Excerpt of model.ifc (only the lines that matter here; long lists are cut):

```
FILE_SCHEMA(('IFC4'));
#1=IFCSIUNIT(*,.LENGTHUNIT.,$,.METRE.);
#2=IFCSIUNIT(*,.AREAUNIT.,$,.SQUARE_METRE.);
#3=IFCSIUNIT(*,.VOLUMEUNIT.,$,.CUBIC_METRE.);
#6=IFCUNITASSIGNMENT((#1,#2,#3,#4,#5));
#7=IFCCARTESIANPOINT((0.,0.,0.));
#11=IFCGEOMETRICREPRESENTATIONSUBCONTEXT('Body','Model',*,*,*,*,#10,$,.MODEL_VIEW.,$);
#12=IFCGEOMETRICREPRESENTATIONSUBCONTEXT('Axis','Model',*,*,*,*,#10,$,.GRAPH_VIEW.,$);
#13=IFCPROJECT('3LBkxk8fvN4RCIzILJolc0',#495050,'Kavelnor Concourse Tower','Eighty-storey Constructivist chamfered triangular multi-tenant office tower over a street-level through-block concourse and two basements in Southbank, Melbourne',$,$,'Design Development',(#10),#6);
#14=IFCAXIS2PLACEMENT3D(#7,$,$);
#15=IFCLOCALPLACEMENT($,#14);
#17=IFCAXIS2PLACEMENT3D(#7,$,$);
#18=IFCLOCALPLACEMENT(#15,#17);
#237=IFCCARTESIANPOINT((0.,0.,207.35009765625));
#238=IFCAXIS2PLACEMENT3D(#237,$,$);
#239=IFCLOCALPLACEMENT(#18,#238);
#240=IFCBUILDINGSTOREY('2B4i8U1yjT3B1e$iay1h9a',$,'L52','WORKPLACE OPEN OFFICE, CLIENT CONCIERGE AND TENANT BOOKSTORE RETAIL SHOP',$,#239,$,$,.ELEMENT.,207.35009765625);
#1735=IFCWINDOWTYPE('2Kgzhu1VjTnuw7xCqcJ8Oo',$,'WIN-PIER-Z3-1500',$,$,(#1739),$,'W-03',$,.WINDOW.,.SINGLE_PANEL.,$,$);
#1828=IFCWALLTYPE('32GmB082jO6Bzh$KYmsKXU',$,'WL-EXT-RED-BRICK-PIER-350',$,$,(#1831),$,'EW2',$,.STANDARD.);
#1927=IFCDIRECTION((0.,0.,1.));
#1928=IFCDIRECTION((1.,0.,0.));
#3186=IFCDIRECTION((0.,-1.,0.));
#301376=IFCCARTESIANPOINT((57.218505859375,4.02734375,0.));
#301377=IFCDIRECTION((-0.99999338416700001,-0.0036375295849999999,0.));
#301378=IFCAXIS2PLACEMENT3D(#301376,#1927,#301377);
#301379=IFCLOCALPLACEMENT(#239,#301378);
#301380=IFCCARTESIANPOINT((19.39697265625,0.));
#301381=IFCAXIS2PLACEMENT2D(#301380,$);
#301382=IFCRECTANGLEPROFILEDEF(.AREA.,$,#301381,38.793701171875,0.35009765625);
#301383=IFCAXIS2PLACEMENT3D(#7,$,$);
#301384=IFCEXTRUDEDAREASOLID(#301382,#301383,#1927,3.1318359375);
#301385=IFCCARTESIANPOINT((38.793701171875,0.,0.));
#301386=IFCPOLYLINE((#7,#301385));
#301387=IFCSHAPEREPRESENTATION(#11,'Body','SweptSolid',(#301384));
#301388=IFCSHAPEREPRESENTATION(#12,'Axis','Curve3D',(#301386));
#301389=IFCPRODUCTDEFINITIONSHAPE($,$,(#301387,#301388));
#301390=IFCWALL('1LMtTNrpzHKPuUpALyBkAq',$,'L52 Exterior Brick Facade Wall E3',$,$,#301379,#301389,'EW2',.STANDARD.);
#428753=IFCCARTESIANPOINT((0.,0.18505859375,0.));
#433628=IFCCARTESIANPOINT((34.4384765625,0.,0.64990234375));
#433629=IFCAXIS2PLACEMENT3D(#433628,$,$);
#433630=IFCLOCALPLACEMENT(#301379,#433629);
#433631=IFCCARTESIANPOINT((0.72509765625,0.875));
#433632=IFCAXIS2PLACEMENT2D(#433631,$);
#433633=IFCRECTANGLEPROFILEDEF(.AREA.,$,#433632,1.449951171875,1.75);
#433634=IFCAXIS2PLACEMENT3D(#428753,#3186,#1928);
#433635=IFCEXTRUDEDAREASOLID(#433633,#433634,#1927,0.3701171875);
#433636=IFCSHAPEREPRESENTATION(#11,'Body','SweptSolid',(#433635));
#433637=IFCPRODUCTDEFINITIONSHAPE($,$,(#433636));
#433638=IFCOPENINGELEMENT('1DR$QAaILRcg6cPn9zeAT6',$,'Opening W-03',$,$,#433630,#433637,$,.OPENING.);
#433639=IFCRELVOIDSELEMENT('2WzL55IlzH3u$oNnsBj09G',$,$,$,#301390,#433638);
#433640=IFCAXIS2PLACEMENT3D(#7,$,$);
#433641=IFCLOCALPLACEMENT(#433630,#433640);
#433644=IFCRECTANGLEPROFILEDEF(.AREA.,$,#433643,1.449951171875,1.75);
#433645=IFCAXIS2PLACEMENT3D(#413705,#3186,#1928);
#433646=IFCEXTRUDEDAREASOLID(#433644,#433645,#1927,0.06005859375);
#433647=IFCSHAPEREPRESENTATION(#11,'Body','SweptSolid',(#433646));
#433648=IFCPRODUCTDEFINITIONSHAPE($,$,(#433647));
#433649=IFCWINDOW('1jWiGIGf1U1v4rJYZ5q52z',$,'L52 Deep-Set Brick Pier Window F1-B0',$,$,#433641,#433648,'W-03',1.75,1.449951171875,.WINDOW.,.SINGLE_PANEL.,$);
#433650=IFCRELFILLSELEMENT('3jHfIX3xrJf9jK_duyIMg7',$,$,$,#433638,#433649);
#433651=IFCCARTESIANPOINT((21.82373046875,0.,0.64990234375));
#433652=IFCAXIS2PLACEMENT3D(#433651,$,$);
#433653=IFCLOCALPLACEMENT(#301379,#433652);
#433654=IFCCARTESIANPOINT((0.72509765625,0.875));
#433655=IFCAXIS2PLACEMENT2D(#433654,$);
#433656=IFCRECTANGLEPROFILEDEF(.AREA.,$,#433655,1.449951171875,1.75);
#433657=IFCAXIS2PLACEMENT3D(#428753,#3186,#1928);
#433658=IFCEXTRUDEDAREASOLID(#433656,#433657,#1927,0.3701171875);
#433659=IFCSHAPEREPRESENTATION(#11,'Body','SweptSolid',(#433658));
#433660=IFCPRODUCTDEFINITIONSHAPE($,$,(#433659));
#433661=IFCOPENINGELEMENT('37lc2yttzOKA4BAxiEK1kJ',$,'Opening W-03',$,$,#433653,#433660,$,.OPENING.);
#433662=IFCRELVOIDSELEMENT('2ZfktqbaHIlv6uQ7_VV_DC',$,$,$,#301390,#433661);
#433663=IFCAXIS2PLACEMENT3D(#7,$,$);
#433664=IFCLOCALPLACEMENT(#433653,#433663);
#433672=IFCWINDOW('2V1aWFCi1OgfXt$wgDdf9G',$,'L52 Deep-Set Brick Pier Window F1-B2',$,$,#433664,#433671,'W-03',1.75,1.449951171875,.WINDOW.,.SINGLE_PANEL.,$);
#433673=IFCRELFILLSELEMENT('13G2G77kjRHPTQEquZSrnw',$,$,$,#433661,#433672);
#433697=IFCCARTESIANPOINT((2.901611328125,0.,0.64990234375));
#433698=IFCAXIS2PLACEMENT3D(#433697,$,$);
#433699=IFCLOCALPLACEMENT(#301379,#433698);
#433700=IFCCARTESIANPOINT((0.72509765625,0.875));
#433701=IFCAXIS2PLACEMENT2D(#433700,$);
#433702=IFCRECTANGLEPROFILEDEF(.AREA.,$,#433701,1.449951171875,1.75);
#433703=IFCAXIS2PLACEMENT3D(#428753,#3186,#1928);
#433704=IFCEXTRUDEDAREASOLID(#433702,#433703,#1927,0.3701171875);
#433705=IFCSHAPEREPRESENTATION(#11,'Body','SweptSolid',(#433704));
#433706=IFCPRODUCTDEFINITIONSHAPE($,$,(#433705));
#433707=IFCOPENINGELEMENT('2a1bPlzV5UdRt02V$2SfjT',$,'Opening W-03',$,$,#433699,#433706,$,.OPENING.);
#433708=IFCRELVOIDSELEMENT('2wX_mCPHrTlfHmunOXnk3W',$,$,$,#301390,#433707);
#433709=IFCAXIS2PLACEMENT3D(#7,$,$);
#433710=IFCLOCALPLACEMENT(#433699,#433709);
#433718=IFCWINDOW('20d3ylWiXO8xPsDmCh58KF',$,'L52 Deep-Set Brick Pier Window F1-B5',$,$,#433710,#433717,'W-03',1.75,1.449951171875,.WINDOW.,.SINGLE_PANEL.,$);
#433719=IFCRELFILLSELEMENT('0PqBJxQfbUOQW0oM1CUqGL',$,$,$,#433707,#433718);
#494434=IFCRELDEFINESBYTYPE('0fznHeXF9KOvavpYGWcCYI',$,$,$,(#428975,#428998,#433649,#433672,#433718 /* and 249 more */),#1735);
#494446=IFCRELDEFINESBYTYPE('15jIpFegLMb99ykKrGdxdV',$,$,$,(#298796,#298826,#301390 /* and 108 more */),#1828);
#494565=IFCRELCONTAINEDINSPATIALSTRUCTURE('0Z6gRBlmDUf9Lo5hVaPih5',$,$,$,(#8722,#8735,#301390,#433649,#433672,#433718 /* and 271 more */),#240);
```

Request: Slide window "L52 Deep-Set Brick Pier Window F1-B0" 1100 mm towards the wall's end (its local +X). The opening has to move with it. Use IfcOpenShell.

```python
import ifcopenshell
import ifcopenshell.api.geometry
import ifcopenshell.util.placement

model = ifcopenshell.open("model.ifc")

window = model.by_id(433649)
opening = window.FillsVoids[0].RelatingOpeningElement
wall = opening.VoidsElements[0].RelatingBuildingElement

wall_matrix = ifcopenshell.util.placement.get_local_placement(wall.ObjectPlacement)
shift = wall_matrix[:3, 0] * 1.1
before = ifcopenshell.util.placement.get_local_placement(window.ObjectPlacement)[:3, 3].copy()

# The window is placed relative to its opening, so it follows when the opening moves.
matrix = ifcopenshell.util.placement.get_local_placement(opening.ObjectPlacement)
matrix[:3, 3] += shift
ifcopenshell.api.geometry.edit_object_placement(
    model, product=opening, matrix=matrix, is_si=False, should_transform_children=True
)

after = ifcopenshell.util.placement.get_local_placement(window.ObjectPlacement)[:3, 3]
print("window moved by", (after - before).round(3) + 0.0)

model.write("model-out.ifc")
```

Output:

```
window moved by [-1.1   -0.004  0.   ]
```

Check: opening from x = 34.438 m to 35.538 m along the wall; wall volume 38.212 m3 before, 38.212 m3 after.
